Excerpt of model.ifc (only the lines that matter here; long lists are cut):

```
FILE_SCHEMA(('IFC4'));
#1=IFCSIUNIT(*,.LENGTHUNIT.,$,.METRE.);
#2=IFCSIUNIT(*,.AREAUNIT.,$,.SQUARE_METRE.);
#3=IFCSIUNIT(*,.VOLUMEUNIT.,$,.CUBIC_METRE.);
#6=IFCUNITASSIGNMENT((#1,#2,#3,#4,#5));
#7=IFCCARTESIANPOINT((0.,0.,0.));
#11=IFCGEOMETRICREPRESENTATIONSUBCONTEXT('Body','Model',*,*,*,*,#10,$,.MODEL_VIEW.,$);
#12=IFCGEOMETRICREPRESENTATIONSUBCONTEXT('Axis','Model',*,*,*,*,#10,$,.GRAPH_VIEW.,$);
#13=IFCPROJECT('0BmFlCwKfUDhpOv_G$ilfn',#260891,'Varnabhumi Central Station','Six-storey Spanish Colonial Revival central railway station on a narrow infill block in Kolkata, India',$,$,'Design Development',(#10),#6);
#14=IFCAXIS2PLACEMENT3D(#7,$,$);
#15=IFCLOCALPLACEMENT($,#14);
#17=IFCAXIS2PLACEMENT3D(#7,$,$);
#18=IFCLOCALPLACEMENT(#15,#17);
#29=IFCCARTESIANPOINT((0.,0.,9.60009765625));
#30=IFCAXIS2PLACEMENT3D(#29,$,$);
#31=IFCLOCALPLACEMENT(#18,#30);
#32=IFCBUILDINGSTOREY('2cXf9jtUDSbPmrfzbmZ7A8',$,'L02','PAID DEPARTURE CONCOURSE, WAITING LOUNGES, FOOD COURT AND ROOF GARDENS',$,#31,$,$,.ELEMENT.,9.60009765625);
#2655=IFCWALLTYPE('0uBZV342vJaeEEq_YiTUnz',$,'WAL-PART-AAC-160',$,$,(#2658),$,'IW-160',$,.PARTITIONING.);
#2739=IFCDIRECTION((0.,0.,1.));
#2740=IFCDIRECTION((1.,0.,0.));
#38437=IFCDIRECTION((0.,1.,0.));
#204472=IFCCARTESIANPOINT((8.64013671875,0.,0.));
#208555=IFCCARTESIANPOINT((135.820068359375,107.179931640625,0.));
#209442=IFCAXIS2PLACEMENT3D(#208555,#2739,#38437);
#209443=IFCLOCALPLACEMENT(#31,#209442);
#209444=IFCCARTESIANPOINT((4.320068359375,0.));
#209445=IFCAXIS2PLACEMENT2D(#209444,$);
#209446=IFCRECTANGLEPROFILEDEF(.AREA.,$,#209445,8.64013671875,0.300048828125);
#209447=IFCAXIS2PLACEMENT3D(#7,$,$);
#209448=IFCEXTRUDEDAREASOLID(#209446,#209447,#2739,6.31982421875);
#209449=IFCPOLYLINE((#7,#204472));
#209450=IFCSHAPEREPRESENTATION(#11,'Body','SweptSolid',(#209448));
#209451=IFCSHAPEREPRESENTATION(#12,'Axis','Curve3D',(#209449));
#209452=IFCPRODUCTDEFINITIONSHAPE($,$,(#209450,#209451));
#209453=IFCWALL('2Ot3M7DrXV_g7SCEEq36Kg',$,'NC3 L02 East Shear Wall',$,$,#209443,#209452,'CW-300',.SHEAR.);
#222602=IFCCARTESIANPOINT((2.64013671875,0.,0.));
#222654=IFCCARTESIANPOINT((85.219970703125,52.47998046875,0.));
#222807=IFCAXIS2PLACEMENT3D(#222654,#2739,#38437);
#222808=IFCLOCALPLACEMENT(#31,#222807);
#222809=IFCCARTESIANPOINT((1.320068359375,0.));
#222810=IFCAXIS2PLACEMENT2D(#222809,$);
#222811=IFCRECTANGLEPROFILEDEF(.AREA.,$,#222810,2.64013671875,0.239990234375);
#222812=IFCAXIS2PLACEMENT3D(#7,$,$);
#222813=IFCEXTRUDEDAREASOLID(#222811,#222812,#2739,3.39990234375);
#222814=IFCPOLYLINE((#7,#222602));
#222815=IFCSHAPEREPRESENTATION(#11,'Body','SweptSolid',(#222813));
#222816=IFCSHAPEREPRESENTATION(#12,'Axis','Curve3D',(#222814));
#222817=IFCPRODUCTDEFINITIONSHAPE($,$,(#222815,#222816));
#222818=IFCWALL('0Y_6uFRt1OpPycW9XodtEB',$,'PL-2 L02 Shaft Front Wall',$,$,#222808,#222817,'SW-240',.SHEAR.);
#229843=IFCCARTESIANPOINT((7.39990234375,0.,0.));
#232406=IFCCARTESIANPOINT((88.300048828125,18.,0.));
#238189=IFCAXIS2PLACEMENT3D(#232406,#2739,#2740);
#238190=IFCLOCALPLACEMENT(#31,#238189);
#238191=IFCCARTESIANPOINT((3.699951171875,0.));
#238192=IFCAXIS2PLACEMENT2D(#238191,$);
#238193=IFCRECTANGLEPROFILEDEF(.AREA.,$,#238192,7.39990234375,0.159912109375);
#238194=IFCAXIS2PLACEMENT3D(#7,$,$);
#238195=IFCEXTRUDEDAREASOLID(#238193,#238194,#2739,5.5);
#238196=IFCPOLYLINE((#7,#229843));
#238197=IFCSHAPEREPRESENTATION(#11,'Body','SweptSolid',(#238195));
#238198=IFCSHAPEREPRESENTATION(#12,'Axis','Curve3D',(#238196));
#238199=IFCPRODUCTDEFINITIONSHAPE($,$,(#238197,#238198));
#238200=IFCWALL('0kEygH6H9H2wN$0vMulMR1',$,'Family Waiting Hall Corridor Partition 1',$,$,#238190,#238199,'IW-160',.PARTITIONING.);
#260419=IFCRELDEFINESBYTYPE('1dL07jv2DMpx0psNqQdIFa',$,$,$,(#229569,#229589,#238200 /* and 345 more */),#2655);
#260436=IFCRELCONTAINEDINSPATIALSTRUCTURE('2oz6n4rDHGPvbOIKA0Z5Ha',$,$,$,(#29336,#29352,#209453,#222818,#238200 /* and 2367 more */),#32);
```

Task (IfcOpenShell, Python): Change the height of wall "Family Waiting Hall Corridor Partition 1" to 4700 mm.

```python
import ifcopenshell
import ifcopenshell.geom
import ifcopenshell.util.representation
import ifcopenshell.util.shape

model = ifcopenshell.open("model.ifc")
settings = ifcopenshell.geom.settings()


def volume(element):
    """Net volume in cubic metres, openings subtracted."""
    shape = ifcopenshell.geom.create_shape(settings, element)
    return ifcopenshell.util.shape.get_volume(shape.geometry)


wall = model.by_guid("0kEygH6H9H2wN$0vMulMR1")
before = volume(wall)

body = ifcopenshell.util.representation.get_representation(wall, "Model", "Body")
solid = body.Items[0]
old_height = solid.Depth
solid.Depth = 4.7
after = volume(wall)

print(f"height {old_height:g} -> {solid.Depth:g}, volume {before:.3f} -> {after:.3f} m3")

model.write("model_v2.ifc")
```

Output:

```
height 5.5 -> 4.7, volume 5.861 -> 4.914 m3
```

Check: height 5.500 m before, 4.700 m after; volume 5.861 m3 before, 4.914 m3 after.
